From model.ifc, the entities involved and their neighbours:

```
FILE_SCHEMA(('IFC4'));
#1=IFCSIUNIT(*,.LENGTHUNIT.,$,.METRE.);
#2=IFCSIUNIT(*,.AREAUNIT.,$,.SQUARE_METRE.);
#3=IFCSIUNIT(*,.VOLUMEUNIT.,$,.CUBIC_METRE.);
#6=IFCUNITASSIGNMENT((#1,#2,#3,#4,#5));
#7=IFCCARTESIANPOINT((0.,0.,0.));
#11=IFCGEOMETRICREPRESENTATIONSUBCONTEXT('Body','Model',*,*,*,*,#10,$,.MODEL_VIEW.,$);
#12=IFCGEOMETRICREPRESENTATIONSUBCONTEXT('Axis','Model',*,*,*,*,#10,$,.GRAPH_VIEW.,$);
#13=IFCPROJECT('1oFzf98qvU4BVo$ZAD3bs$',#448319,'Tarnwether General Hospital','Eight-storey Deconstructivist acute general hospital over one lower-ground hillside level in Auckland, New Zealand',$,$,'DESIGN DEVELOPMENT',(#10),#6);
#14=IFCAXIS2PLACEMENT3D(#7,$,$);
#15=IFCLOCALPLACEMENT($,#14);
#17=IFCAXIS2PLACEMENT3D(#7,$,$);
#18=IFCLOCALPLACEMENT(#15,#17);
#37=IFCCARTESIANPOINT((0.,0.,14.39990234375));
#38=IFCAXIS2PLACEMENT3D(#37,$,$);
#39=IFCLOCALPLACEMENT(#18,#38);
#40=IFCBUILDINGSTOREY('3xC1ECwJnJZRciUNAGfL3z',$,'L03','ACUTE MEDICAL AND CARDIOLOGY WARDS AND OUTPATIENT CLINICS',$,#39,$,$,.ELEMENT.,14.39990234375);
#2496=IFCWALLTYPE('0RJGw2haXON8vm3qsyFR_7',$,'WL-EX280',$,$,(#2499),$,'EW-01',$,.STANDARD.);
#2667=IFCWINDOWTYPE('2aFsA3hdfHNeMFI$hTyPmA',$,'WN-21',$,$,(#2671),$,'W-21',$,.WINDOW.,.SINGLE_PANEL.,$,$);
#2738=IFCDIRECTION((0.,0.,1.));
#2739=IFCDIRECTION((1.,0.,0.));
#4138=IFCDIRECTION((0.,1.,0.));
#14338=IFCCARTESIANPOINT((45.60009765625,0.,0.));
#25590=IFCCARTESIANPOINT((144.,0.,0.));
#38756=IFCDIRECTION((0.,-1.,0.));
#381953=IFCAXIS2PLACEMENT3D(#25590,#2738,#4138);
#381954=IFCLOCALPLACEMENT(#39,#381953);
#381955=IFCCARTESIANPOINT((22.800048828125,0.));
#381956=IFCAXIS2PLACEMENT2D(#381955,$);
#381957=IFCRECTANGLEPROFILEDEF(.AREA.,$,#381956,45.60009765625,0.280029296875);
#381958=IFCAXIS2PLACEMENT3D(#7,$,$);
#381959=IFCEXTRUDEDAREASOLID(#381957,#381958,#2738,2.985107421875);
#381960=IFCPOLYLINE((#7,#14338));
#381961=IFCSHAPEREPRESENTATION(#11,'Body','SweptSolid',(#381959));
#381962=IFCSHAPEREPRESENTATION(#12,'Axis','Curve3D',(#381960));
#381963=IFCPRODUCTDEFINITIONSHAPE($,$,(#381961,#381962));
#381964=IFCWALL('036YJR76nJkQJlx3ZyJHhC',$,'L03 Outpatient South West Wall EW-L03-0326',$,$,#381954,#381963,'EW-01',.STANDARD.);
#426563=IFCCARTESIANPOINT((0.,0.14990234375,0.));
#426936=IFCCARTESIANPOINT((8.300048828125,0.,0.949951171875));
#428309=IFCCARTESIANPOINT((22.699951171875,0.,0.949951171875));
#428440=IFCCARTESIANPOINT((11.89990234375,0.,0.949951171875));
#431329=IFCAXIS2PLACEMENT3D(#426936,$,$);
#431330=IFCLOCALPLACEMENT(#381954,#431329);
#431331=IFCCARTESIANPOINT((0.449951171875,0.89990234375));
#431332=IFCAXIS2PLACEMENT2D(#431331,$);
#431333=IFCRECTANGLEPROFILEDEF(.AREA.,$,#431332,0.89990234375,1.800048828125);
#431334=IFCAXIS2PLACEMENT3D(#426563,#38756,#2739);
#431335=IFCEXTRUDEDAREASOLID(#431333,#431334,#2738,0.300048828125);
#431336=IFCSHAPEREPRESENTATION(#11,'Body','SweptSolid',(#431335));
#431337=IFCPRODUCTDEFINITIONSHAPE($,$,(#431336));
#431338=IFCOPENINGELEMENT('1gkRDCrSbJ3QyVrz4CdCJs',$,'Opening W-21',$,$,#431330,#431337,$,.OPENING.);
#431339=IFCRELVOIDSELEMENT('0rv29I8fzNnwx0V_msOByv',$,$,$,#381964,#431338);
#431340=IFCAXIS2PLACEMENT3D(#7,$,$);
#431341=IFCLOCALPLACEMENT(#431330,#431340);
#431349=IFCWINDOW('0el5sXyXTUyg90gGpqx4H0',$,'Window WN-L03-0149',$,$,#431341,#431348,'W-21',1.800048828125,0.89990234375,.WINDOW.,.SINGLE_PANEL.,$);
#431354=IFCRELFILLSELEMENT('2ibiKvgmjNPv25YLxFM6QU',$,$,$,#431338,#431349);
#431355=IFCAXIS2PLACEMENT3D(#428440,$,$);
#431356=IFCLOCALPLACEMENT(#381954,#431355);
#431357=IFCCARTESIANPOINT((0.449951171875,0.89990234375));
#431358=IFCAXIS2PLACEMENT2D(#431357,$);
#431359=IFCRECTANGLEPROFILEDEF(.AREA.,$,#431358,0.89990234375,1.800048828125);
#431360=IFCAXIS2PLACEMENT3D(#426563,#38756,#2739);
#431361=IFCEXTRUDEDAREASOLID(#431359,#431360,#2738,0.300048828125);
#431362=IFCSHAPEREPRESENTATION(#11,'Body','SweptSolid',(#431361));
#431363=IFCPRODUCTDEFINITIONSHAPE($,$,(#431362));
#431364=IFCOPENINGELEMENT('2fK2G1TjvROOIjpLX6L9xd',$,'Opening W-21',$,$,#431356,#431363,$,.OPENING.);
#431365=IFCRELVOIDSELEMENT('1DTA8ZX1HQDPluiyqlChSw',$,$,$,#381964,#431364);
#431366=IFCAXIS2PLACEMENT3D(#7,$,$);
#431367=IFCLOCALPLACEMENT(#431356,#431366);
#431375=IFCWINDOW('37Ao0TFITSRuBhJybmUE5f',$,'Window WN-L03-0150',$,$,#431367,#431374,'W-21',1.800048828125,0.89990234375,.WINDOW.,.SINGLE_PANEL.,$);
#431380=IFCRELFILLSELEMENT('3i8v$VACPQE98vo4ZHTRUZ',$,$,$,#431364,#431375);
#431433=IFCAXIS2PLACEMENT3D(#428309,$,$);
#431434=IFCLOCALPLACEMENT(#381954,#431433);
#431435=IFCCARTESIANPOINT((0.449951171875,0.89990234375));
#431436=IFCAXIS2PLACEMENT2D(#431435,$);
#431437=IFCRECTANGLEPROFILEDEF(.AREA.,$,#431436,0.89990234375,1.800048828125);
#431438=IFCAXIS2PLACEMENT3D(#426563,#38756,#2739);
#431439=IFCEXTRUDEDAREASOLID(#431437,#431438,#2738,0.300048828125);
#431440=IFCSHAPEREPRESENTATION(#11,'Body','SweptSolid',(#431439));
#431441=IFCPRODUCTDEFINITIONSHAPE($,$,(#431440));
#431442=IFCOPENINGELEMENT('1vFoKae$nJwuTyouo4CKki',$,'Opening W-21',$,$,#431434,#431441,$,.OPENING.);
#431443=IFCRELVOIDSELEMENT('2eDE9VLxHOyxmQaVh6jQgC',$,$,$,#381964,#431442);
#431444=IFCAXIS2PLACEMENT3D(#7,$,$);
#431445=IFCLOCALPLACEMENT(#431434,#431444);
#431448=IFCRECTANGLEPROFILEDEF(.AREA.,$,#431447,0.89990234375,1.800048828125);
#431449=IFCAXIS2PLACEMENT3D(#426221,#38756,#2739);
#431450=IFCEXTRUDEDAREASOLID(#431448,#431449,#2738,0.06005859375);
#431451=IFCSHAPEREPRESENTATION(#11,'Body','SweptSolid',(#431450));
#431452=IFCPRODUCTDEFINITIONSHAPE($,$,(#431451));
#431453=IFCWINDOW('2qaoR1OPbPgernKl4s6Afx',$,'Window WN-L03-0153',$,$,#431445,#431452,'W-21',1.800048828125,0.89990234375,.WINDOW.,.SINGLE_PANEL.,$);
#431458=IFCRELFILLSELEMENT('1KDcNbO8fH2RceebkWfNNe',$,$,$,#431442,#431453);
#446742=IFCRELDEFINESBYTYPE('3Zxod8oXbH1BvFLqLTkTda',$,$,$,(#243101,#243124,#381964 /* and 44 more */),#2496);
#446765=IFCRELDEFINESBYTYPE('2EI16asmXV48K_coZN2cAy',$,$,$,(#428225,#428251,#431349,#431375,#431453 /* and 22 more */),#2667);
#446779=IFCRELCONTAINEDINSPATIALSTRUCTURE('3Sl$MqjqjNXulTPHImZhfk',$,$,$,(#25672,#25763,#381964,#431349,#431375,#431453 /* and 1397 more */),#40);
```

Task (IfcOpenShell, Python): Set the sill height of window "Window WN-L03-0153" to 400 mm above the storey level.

```python
import numpy as np
import ifcopenshell
import ifcopenshell.api.geometry
import ifcopenshell.geom
import ifcopenshell.util.element
import ifcopenshell.util.placement
import ifcopenshell.util.shape
import ifcopenshell.util.unit

model = ifcopenshell.open("model.ifc")
unit_scale = ifcopenshell.util.unit.calculate_unit_scale(model)

window = model.by_guid("2qaoR1OPbPgernKl4s6Afx")
opening = window.FillsVoids[0].RelatingOpeningElement
storey = ifcopenshell.util.element.get_container(window, ifc_class="IfcBuildingStorey")
level = ifcopenshell.util.placement.get_local_placement(storey.ObjectPlacement)[2, 3]

# The opening's origin need not be at the sill, so measure its lowest point.
shape = ifcopenshell.geom.create_shape(ifcopenshell.geom.settings(), opening)
bottom = ifcopenshell.util.shape.get_shape_bottom_elevation(shape, shape.geometry) / unit_scale
dz = level + 0.4 / unit_scale - bottom

shift = np.array([0.0, 0.0, dz])
# The window is placed relative to its opening, so it follows when the opening moves.
matrix = ifcopenshell.util.placement.get_local_placement(opening.ObjectPlacement)
matrix[:3, 3] += shift
ifcopenshell.api.geometry.edit_object_placement(
    model, product=opening, matrix=matrix, is_si=False, should_transform_children=True
)

print(f"moved by {dz * unit_scale:+.3f} m")

model.write("model_rev.ifc")
```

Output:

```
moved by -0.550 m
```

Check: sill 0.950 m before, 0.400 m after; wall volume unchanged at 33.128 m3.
